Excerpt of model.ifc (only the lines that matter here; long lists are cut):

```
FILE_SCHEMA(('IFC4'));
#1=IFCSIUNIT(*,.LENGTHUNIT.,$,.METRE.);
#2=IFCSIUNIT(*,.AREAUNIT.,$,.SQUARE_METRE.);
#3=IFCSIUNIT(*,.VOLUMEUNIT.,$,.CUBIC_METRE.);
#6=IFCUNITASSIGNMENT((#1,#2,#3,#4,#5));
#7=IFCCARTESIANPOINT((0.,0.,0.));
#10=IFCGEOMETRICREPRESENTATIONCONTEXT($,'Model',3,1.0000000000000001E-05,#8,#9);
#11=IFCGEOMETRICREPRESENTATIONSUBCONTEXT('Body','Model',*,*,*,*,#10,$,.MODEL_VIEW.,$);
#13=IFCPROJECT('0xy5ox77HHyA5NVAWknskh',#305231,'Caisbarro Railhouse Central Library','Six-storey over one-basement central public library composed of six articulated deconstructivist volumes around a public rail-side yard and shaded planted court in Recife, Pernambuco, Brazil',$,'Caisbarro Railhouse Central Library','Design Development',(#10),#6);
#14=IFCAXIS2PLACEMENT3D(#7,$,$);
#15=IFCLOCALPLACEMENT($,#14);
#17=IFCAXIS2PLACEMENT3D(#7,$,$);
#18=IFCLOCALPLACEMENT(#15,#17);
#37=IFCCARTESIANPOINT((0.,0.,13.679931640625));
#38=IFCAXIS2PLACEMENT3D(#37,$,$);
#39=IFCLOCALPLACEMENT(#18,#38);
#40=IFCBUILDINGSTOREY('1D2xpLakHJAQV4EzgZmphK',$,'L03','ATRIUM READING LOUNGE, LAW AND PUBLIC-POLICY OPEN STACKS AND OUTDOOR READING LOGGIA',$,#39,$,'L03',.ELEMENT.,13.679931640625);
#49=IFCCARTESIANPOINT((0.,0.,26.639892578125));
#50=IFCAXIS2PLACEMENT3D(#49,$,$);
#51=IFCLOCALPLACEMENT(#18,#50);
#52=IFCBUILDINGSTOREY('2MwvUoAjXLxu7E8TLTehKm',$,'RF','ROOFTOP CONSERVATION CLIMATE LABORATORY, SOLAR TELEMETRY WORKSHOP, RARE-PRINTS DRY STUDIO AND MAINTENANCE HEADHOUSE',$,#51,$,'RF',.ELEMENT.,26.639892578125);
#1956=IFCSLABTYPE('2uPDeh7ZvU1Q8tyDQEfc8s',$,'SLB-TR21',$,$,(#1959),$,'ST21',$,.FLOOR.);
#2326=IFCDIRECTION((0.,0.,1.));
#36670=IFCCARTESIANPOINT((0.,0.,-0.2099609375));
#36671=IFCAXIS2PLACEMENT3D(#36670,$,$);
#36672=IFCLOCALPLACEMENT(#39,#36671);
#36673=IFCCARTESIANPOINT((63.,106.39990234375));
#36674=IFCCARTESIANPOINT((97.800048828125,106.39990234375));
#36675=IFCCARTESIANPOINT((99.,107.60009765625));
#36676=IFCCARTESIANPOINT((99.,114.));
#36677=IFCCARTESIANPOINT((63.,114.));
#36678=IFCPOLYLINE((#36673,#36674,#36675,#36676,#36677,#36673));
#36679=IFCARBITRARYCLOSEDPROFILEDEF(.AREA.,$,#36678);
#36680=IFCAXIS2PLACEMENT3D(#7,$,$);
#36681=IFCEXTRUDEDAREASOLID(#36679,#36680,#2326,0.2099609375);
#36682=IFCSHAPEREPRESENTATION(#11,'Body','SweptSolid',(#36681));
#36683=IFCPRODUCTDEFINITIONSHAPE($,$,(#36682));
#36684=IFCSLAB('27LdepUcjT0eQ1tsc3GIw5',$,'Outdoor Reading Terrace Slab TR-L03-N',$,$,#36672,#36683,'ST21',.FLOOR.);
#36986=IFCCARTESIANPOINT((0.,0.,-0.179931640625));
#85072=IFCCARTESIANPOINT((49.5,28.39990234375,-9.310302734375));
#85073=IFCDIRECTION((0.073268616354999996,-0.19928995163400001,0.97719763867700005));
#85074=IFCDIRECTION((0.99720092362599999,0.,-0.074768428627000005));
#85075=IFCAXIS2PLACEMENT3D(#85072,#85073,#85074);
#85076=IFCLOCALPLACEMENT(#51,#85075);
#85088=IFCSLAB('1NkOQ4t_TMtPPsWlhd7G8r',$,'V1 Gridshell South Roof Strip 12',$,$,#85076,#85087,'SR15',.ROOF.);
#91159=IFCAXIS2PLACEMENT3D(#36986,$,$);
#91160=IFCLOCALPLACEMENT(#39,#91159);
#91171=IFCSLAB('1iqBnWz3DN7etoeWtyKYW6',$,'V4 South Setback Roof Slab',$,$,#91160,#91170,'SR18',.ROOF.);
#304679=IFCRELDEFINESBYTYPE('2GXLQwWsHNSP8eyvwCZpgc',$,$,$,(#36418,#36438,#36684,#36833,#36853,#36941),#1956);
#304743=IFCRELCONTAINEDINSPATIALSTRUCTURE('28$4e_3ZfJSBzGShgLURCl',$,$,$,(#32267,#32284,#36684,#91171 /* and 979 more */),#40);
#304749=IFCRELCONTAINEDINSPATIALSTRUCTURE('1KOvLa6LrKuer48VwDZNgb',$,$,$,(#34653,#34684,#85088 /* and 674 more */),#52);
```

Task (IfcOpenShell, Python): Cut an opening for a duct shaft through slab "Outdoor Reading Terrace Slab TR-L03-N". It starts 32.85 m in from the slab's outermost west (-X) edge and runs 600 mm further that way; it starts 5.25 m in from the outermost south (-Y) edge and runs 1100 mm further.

```python
import numpy as np
import ifcopenshell
import ifcopenshell.api.feature
import ifcopenshell.api.geometry
import ifcopenshell.api.root
import ifcopenshell.geom
import ifcopenshell.util.placement
import ifcopenshell.util.representation
import ifcopenshell.util.shape
import ifcopenshell.util.unit

model = ifcopenshell.open("model.ifc")
unit_scale = ifcopenshell.util.unit.calculate_unit_scale(model)
settings = ifcopenshell.geom.settings()


def volume(element):
    """Net volume in cubic metres, openings subtracted."""
    shape = ifcopenshell.geom.create_shape(settings, element)
    return ifcopenshell.util.shape.get_volume(shape.geometry)


slab = model.by_guid("27LdepUcjT0eQ1tsc3GIw5")
before = volume(slab)

# Extent in the slab's own axes, in metres. The edges named are its -X and -Y sides.
slab_shape = ifcopenshell.geom.create_shape(settings, slab)
vertices = ifcopenshell.util.shape.get_vertices(slab_shape.geometry)
x_min, y_min, bottom = vertices.min(axis=0)
top = vertices[:, 2].max()

opening = ifcopenshell.api.root.create_entity(model, ifc_class="IfcOpeningElement", name="Duct shaft opening", predefined_type="OPENING")
context = ifcopenshell.util.representation.get_context(model, "Model", "Body", "MODEL_VIEW")
width, depth = 0.6, 1.1
outline = [(0.0, 0.0), (width, 0.0), (width, depth), (0.0, depth), (0.0, 0.0)]
# Overshoot both faces by 50 mm so the cut is clean.
shape = ifcopenshell.api.geometry.add_slab_representation(
    model, context=context, depth=top - bottom + 0.1, polyline=outline
)
ifcopenshell.api.geometry.assign_representation(model, product=opening, representation=shape)

matrix = ifcopenshell.util.placement.get_local_placement(slab.ObjectPlacement)
matrix[:, 3] = matrix @ np.append(np.array([x_min + 32.85, y_min + 5.25, bottom - 0.05]) / unit_scale, 1.0)
ifcopenshell.api.geometry.edit_object_placement(model, product=opening, matrix=matrix, is_si=False)
ifcopenshell.api.feature.add_feature(model, feature=opening, element=slab)

after = volume(slab)

print(f"slab volume {before:.3f} -> {after:.3f} m3")

model.write("model_v2.ifc")
```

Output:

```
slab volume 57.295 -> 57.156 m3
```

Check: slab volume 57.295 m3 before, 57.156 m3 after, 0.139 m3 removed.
